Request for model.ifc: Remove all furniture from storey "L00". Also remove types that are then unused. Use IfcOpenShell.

First a look at what the model holds.

```python
import ifcopenshell
import ifcopenshell.util.element

model = ifcopenshell.open("model.ifc")
print(model.schema)
storey = next(s for s in model.by_type("IfcBuildingStorey") if s.Name == "L00")
furniture = [e for e in ifcopenshell.util.element.get_decomposition(storey) if e.is_a("IfcFurnishingElement")]
seen = {}
for e in furniture:
    element_type = ifcopenshell.util.element.get_type(e)
    name = element_type.Name if element_type not in (None, e) else None
    seen[name] = seen.get(name, 0) + 1
for name, count in sorted(seen.items(), key=str):
    print(count, "x", name)
```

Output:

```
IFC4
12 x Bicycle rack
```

```python
import ifcopenshell
import ifcopenshell.api.root
import ifcopenshell.util.element

model = ifcopenshell.open("model.ifc")

storey = next(s for s in model.by_type("IfcBuildingStorey") if s.Name == "L00")
furniture = [e for e in ifcopenshell.util.element.get_decomposition(storey) if e.is_a("IfcFurnishingElement")]
types = {ifcopenshell.util.element.get_type(e) for e in furniture} - {None, *furniture}

for e in furniture:
    ifcopenshell.api.root.remove_product(model, product=e)
print(len(furniture), "removed")

unused = [t for t in types if not ifcopenshell.util.element.get_types(t)]
for t in unused:
    ifcopenshell.api.root.remove_product(model, product=t)
print(len(unused), "unused types removed")

model.write("model_edited.ifc")
```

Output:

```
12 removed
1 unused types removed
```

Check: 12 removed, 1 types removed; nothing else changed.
